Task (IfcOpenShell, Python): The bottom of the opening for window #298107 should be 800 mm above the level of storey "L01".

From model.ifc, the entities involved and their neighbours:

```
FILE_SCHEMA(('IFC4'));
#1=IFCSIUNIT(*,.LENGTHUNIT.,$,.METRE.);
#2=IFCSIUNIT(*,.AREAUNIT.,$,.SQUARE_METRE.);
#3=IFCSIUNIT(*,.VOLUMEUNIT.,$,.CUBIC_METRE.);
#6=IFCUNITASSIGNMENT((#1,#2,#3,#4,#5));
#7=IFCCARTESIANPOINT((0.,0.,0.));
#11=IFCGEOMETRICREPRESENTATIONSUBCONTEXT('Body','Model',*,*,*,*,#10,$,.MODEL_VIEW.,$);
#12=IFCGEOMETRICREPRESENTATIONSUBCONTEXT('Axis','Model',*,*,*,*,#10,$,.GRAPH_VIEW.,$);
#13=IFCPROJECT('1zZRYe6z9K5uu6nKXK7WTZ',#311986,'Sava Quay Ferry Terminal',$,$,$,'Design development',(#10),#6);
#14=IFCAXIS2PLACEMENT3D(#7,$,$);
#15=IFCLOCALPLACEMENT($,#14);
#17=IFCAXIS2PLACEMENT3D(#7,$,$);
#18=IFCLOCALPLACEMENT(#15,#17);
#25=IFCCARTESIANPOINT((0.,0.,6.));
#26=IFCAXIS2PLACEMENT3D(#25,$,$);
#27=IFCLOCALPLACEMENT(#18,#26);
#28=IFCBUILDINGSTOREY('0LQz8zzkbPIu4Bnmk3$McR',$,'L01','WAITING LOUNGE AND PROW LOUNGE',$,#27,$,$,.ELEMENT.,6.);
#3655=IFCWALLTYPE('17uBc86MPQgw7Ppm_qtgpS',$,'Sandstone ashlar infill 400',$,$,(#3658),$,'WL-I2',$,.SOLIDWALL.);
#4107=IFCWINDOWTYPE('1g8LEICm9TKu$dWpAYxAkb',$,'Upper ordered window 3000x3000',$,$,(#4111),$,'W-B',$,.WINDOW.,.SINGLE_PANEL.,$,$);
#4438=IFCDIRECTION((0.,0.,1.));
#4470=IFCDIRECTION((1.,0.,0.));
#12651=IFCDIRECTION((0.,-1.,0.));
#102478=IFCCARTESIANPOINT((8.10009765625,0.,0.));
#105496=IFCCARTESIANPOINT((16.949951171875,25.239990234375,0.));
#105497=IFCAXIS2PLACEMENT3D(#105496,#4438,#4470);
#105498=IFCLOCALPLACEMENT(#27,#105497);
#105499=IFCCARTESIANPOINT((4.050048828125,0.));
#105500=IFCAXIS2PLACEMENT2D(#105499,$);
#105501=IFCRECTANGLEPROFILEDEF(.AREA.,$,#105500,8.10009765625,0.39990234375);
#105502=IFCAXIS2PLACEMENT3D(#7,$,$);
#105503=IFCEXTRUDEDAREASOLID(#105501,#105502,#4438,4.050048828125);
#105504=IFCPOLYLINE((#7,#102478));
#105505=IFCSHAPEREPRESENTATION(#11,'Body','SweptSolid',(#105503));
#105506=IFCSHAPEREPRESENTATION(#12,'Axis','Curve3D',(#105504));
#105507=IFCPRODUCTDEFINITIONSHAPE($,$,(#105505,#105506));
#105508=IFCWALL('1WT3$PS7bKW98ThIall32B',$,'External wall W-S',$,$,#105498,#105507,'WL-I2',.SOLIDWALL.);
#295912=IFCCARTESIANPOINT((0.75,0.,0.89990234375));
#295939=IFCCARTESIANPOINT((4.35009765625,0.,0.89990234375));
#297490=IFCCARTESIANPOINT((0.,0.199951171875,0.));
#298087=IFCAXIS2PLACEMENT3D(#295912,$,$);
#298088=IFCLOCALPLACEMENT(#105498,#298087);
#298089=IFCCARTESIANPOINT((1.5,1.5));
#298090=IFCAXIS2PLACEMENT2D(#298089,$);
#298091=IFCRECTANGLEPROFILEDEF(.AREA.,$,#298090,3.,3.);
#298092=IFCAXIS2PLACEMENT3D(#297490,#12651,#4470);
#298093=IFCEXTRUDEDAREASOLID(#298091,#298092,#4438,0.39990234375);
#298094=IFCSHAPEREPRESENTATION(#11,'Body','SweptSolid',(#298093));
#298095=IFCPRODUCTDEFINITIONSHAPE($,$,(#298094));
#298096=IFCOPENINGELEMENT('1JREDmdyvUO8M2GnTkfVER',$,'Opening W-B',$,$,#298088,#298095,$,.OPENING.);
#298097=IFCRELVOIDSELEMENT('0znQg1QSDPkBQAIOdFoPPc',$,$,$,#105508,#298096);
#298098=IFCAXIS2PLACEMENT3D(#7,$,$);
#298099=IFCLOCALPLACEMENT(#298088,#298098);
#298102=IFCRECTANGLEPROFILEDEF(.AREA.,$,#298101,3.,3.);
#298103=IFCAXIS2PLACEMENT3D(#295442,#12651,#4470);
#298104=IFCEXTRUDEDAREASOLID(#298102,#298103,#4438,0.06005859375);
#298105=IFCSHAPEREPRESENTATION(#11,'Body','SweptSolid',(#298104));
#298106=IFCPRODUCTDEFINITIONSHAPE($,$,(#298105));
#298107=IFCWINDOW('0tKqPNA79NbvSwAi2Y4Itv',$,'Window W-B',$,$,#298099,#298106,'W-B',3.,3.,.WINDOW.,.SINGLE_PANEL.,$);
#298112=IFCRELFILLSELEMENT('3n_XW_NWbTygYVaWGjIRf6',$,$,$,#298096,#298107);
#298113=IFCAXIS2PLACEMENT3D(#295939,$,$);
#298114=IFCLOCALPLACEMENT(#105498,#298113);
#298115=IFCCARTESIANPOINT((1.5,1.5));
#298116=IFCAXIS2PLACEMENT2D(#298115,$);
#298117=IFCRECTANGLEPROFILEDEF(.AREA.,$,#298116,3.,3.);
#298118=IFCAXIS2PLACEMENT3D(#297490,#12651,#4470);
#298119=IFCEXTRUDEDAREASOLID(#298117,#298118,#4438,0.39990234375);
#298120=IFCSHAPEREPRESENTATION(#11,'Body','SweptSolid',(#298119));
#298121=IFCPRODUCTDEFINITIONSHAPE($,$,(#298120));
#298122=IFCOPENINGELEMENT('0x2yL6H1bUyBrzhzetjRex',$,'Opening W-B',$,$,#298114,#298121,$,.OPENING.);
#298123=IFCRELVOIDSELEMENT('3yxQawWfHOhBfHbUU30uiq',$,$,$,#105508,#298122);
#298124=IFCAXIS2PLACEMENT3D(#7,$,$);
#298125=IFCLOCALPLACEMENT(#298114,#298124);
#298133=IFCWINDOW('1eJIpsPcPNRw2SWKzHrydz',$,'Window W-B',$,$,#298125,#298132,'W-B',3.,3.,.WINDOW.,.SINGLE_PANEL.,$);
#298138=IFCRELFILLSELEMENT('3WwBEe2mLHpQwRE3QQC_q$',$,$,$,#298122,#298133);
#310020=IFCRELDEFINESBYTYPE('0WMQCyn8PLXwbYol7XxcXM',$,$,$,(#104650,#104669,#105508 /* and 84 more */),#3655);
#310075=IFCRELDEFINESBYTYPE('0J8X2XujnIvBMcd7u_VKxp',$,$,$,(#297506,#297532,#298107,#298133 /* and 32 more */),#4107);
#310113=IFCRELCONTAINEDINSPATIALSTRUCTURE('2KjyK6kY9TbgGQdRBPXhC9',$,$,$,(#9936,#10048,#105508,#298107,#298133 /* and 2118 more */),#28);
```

```python
import numpy as np
import ifcopenshell
import ifcopenshell.api.geometry
import ifcopenshell.geom
import ifcopenshell.util.element
import ifcopenshell.util.placement
import ifcopenshell.util.shape
import ifcopenshell.util.unit

model = ifcopenshell.open("model.ifc")
unit_scale = ifcopenshell.util.unit.calculate_unit_scale(model)

window = model.by_guid("0tKqPNA79NbvSwAi2Y4Itv")
opening = window.FillsVoids[0].RelatingOpeningElement
storey = ifcopenshell.util.element.get_container(window, ifc_class="IfcBuildingStorey")
level = ifcopenshell.util.placement.get_local_placement(storey.ObjectPlacement)[2, 3]

# The opening's origin need not be at the sill, so measure its lowest point.
shape = ifcopenshell.geom.create_shape(ifcopenshell.geom.settings(), opening)
bottom = ifcopenshell.util.shape.get_shape_bottom_elevation(shape, shape.geometry) / unit_scale
dz = level + 0.8 - bottom

shift = np.array([0.0, 0.0, dz])
# The window is placed relative to its opening, so it follows when the opening moves.
matrix = ifcopenshell.util.placement.get_local_placement(opening.ObjectPlacement)
matrix[:3, 3] += shift
ifcopenshell.api.geometry.edit_object_placement(
    model, product=opening, matrix=matrix, is_si=False, should_transform_children=True
)

print(f"moved by {dz * unit_scale:+.3f} m")

model.write("model_edited.ifc")
```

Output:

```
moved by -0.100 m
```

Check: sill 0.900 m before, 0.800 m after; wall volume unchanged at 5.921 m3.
